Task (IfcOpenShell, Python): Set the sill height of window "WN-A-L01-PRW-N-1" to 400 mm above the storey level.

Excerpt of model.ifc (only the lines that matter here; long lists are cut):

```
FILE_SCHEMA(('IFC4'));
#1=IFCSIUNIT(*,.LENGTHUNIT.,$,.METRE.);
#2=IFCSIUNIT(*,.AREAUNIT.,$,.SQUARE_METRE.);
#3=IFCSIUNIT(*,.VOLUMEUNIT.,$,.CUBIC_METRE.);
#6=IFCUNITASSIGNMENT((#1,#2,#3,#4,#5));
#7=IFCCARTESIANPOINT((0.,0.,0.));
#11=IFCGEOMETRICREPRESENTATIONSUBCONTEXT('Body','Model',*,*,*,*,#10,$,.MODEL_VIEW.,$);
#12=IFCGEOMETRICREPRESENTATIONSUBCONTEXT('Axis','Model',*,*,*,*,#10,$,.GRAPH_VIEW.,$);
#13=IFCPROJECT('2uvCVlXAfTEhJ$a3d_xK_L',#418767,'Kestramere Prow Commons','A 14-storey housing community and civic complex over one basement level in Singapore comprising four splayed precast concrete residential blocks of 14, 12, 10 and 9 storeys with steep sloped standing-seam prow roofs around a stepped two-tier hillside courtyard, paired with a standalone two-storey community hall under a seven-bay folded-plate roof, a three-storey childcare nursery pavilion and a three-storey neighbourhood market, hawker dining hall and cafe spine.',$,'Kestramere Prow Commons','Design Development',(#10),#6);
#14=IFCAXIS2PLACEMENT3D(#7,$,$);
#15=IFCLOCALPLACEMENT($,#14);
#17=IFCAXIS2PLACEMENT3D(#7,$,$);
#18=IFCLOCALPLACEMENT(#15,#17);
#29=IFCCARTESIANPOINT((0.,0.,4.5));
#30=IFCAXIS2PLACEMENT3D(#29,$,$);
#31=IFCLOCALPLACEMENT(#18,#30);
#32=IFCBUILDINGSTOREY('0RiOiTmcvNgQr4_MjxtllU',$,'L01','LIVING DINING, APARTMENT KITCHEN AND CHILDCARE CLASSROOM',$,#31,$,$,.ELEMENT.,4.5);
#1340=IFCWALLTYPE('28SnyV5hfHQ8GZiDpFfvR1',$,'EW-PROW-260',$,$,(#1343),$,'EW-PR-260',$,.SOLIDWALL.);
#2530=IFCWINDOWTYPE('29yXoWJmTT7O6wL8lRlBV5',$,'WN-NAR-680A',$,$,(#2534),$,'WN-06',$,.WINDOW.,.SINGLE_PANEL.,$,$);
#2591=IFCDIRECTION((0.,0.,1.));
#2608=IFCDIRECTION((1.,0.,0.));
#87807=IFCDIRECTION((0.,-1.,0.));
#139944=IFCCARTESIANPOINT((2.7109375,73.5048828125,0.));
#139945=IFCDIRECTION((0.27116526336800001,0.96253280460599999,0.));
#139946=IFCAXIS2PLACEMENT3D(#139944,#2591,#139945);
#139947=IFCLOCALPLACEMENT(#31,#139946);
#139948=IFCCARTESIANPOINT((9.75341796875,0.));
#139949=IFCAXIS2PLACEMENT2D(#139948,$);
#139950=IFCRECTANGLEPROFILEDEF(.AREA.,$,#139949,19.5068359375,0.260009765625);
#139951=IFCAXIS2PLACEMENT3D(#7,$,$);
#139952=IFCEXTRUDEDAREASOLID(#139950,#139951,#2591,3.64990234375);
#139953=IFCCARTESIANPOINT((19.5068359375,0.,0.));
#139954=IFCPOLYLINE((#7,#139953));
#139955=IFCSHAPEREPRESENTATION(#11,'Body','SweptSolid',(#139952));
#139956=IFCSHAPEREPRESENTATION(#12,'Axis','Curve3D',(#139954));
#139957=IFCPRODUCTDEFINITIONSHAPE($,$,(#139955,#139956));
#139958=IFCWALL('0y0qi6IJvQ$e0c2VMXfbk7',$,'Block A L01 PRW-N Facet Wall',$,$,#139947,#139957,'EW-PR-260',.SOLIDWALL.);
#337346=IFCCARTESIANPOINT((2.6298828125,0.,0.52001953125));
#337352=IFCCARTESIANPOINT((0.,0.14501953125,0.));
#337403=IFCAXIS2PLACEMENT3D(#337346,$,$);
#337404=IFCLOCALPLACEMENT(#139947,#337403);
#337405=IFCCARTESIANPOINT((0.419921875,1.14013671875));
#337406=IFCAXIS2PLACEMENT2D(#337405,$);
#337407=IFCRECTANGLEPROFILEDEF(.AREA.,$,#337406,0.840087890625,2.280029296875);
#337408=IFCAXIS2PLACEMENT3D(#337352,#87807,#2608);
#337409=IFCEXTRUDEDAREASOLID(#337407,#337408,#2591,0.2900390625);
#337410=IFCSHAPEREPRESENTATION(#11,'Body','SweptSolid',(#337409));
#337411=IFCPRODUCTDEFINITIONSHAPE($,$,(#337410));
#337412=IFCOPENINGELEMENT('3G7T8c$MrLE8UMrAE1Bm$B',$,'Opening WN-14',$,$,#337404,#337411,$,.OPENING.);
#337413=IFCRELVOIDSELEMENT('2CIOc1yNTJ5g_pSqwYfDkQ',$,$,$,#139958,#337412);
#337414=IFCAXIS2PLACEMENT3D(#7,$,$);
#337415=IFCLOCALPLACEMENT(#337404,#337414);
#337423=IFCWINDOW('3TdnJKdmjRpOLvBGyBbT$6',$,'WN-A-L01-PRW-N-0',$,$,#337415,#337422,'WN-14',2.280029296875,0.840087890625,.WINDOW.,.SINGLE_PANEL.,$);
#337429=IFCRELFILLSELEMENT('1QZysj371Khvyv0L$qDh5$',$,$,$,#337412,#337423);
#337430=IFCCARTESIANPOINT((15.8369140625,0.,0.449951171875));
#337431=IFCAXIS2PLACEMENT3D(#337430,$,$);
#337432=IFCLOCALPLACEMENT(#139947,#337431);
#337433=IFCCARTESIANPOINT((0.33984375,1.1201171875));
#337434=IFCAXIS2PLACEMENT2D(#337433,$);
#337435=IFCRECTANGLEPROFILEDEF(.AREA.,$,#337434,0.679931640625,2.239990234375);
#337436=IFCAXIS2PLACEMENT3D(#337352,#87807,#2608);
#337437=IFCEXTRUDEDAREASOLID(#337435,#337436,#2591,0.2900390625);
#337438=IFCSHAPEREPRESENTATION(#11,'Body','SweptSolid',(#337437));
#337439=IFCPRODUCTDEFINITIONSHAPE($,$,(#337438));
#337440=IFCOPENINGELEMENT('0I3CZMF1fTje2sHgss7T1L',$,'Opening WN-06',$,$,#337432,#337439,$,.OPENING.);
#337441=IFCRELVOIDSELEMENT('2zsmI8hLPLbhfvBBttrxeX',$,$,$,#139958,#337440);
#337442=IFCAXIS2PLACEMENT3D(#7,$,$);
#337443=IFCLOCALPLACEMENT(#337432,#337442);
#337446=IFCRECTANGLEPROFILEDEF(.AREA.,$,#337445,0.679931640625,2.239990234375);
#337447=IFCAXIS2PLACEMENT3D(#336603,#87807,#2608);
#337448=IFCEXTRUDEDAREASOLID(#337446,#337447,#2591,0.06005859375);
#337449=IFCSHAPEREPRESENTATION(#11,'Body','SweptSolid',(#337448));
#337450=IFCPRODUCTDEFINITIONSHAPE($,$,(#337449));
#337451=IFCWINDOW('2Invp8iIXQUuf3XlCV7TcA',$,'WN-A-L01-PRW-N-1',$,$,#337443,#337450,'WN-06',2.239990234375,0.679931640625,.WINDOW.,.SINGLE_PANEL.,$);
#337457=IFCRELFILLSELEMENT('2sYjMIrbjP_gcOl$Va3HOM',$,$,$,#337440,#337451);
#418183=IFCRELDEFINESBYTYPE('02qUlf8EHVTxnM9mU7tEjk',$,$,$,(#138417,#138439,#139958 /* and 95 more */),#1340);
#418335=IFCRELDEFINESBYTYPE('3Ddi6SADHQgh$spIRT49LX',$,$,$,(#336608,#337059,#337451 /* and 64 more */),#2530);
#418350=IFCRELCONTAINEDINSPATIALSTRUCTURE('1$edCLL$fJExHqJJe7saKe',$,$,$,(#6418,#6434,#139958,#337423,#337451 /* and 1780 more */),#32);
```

```python
import numpy as np
import ifcopenshell
import ifcopenshell.api.geometry
import ifcopenshell.geom
import ifcopenshell.util.element
import ifcopenshell.util.placement
import ifcopenshell.util.shape
import ifcopenshell.util.unit

model = ifcopenshell.open("model.ifc")
unit_scale = ifcopenshell.util.unit.calculate_unit_scale(model)

window = model.by_id(337451)
opening = window.FillsVoids[0].RelatingOpeningElement
storey = ifcopenshell.util.element.get_container(window, ifc_class="IfcBuildingStorey")
level = ifcopenshell.util.placement.get_local_placement(storey.ObjectPlacement)[2, 3]

# The opening's origin need not be at the sill, so measure its lowest point.
shape = ifcopenshell.geom.create_shape(ifcopenshell.geom.settings(), opening)
bottom = ifcopenshell.util.shape.get_shape_bottom_elevation(shape, shape.geometry) / unit_scale
dz = level + 0.4 / unit_scale - bottom

shift = np.array([0.0, 0.0, dz])
# The window is placed relative to its opening, so it follows when the opening moves.
matrix = ifcopenshell.util.placement.get_local_placement(opening.ObjectPlacement)
matrix[:3, 3] += shift
ifcopenshell.api.geometry.edit_object_placement(
    model, product=opening, matrix=matrix, is_si=False, should_transform_children=True
)

print(f"moved by {dz * unit_scale:+.3f} m")

model.write("model-out.ifc")
```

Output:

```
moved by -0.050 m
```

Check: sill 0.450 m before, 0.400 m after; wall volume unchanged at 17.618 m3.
